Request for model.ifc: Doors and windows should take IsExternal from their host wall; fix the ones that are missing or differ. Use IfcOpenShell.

First a look at what the model holds.

```python
import ifcopenshell
import ifcopenshell.util.element

model = ifcopenshell.open("model.ifc")
print(model.schema)
seen = {}
for e in model.by_type("IfcDoor") + model.by_type("IfcWindow"):
    if not e.FillsVoids:
        continue
    host = e.FillsVoids[0].RelatingOpeningElement.VoidsElements[0].RelatingBuildingElement
    own = ifcopenshell.util.element.get_pset(e, f"Pset_{e.is_a()[3:].removesuffix('StandardCase')}Common", "IsExternal")
    wall = ifcopenshell.util.element.get_pset(host, "Pset_WallCommon", "IsExternal")
    seen[e.is_a(), own, wall] = seen.get((e.is_a(), own, wall), 0) + 1
for (cls, own, wall), count in sorted(seen.items(), key=str):
    print(count, cls, "IsExternal:", own, "| host wall:", wall)
```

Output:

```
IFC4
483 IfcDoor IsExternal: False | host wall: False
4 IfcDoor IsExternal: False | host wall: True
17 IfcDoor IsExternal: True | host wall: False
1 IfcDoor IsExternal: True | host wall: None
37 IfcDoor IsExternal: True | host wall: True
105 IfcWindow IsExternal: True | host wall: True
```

```python
import ifcopenshell
import ifcopenshell.api.pset
import ifcopenshell.util.element

model = ifcopenshell.open("model.ifc")

count = 0
for ifc_class, pset_name in (("IfcDoor", "Pset_DoorCommon"), ("IfcWindow", "Pset_WindowCommon")):
    for e in model.by_type(ifc_class):
        if not e.FillsVoids:
            continue
        host = e.FillsVoids[0].RelatingOpeningElement.VoidsElements[0].RelatingBuildingElement
        external = ifcopenshell.util.element.get_pset(host, "Pset_WallCommon", "IsExternal")
        if external is None or ifcopenshell.util.element.get_pset(e, pset_name, "IsExternal") == external:
            continue
        pset = ifcopenshell.api.pset.add_pset(model, product=e, name=pset_name)
        ifcopenshell.api.pset.edit_pset(model, pset=pset, properties={"IsExternal": external})
        count += 1

print(count, "updated")

model.write("model_v2.ifc")
```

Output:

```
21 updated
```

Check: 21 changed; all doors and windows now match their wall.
